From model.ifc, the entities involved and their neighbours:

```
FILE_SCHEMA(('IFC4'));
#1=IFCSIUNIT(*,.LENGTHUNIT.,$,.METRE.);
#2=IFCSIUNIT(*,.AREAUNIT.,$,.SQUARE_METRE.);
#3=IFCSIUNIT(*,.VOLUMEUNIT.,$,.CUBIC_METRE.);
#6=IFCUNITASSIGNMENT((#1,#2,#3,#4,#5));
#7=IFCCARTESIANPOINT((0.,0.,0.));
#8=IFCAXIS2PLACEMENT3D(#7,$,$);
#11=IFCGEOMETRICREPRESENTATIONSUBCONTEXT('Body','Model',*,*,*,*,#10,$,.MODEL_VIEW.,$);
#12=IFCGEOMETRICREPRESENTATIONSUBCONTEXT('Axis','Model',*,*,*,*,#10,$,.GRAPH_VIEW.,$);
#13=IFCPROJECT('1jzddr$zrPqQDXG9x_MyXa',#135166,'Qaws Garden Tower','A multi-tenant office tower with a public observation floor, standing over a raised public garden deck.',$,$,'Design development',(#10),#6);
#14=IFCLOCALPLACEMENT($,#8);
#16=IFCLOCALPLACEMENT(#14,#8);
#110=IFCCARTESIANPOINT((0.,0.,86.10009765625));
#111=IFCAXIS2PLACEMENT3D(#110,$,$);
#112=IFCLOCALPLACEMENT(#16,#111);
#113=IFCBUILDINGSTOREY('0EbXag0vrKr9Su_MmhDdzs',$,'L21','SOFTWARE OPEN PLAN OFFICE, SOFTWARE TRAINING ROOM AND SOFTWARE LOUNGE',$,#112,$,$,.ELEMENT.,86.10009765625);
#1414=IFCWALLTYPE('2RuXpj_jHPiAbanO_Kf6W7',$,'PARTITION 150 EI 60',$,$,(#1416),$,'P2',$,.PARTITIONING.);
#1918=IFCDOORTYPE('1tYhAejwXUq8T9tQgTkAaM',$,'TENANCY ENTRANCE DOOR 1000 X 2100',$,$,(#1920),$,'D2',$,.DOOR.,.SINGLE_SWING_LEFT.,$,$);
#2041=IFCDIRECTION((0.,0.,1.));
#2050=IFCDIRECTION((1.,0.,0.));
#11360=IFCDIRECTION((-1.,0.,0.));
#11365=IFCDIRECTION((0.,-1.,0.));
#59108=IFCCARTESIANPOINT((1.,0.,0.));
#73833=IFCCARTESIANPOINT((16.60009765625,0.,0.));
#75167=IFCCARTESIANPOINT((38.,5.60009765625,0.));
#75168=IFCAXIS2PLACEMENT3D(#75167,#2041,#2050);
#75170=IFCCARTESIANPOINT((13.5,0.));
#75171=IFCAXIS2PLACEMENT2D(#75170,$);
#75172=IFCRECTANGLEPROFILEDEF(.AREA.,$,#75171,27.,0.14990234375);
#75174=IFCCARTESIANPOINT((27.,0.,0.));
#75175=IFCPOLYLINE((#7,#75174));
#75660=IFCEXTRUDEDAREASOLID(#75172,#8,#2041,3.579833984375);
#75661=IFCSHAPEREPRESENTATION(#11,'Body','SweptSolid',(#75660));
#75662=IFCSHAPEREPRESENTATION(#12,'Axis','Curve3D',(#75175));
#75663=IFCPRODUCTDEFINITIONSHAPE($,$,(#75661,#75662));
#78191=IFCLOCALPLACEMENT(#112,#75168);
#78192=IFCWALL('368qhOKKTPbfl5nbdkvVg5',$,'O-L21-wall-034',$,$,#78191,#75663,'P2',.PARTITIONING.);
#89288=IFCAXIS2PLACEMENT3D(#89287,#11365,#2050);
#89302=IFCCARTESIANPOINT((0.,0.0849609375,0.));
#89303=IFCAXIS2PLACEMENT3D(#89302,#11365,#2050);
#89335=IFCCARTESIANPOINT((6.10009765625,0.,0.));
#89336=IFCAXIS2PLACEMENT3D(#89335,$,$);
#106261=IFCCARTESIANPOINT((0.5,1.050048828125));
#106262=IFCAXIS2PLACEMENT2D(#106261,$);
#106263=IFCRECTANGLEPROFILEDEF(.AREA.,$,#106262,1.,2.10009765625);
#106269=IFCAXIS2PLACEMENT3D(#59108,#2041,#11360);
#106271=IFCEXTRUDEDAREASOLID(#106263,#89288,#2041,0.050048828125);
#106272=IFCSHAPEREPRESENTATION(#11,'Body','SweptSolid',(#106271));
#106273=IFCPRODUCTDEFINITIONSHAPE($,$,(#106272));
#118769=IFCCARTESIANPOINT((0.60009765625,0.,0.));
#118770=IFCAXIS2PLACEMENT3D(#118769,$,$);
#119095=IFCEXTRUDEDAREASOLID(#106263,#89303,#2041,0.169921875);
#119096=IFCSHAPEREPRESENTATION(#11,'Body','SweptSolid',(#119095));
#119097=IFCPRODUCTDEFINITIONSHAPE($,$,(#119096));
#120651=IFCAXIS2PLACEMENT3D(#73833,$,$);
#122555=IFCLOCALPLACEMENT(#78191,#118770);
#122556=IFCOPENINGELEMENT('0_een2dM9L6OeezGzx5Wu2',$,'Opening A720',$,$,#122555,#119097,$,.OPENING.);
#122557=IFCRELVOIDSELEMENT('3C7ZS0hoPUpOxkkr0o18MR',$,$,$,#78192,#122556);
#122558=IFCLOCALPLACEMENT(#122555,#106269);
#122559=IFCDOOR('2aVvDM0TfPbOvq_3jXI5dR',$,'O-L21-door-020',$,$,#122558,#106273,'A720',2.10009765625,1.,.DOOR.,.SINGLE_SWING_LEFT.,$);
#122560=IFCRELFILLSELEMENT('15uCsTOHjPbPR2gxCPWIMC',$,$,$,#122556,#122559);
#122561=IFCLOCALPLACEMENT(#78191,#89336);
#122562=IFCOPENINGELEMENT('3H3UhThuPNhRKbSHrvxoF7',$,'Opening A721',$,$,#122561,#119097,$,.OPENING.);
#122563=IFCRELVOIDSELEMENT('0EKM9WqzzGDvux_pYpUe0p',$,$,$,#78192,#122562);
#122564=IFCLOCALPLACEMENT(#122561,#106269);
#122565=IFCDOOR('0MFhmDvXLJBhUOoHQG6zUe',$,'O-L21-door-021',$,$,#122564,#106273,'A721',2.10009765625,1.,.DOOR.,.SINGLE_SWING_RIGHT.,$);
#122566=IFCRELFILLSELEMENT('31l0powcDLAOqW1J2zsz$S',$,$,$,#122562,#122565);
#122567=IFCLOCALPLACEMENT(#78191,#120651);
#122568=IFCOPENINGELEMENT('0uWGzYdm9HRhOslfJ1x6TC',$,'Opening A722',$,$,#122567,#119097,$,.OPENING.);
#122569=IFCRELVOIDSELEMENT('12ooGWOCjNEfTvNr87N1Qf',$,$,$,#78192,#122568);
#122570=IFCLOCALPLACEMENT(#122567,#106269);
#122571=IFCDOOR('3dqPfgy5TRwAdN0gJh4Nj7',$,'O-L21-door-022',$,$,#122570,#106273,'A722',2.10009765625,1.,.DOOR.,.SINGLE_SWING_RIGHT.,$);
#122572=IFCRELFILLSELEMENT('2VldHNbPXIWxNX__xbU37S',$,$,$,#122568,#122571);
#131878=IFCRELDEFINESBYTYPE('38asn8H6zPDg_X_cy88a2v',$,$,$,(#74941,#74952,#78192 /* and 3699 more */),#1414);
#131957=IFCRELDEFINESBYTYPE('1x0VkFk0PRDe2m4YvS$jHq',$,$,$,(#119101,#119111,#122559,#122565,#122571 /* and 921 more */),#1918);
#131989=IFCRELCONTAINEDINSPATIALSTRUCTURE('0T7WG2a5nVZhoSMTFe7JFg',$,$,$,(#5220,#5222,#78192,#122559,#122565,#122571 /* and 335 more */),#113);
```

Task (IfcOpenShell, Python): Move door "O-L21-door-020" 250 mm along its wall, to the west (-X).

```python
import ifcopenshell
import ifcopenshell.api.geometry
import ifcopenshell.util.placement

model = ifcopenshell.open("model.ifc")

door = model.by_id(122559)
opening = door.FillsVoids[0].RelatingOpeningElement
wall = opening.VoidsElements[0].RelatingBuildingElement

wall_matrix = ifcopenshell.util.placement.get_local_placement(wall.ObjectPlacement)
shift = wall_matrix[:3, 0] * -0.25
before = ifcopenshell.util.placement.get_local_placement(door.ObjectPlacement)[:3, 3].copy()

# The door is placed relative to its opening, so it follows when the opening moves.
matrix = ifcopenshell.util.placement.get_local_placement(opening.ObjectPlacement)
matrix[:3, 3] += shift
ifcopenshell.api.geometry.edit_object_placement(
    model, product=opening, matrix=matrix, is_si=False, should_transform_children=True
)

after = ifcopenshell.util.placement.get_local_placement(door.ObjectPlacement)[:3, 3]
print("door moved by", (after - before).round(3) + 0.0)

model.write("model-out.ifc")
```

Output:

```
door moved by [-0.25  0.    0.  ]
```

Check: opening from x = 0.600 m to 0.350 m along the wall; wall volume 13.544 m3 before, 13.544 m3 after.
